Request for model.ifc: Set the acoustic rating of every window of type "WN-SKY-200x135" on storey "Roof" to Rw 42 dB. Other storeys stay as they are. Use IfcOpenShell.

First a look at what the model holds.

```python
import ifcopenshell
import ifcopenshell.util.element

model = ifcopenshell.open("model.ifc")
print(model.schema)
storey = next(s for s in model.by_type("IfcBuildingStorey") if s.Name == "Roof")
windows = [e for e in ifcopenshell.util.element.get_decomposition(storey) if e.is_a("IfcWindow")]
seen = {}
for e in windows:
    element_type = ifcopenshell.util.element.get_type(e)
    key = (element_type.Name if element_type != e and element_type else None, ifcopenshell.util.element.get_pset(e, "Pset_WindowCommon", "AcousticRating"))
    seen[key] = seen.get(key, 0) + 1
for (name, value), count in sorted(seen.items(), key=str):
    print(count, "x", name, "|", value)
```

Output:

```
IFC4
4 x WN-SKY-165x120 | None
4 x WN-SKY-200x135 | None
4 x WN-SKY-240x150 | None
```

```python
import ifcopenshell
import ifcopenshell.api.pset
import ifcopenshell.util.element

model = ifcopenshell.open("model.ifc")

storey = next(s for s in model.by_type("IfcBuildingStorey") if s.Name == "Roof")
windows = [e for e in ifcopenshell.util.element.get_decomposition(storey) if e.is_a("IfcWindow")]

count = 0
for e in windows:
    element_type = ifcopenshell.util.element.get_type(e)
    if element_type in (None, e) or element_type.Name != "WN-SKY-200x135":
        continue
    # add_pset returns the element's existing set when there is one.
    pset = ifcopenshell.api.pset.add_pset(model, product=e, name="Pset_WindowCommon")
    ifcopenshell.api.pset.edit_pset(model, pset=pset, properties={"AcousticRating": "Rw 42 dB"})
    count += 1

print(count, "windows updated")

model.write("model_rev.ifc")
```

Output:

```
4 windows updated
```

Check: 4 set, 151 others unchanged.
